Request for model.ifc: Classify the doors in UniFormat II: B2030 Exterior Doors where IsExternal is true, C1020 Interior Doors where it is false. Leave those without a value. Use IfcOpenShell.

First a look at what the model holds.

```python
import ifcopenshell
import ifcopenshell.util.element

model = ifcopenshell.open("model.ifc")
print(model.schema)
print("classifications:", [c.Name for c in model.by_type("IfcClassification")])
values = [ifcopenshell.util.element.get_pset(e, "Pset_DoorCommon", "IsExternal") for e in model.by_type("IfcDoor")]
for value in (True, False, None):
    print("IsExternal", value, values.count(value))
```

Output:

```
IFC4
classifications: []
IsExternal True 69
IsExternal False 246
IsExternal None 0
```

```python
import ifcopenshell
import ifcopenshell.api.classification
import ifcopenshell.util.element

model = ifcopenshell.open("model.ifc")

system = ifcopenshell.api.classification.add_classification(model, classification="UniFormat II")

doors = model.by_type("IfcDoor")
external = {e: ifcopenshell.util.element.get_pset(e, "Pset_DoorCommon", "IsExternal") for e in doors}
for flag, code, name in ((True, "B2030", "Exterior Doors"), (False, "C1020", "Interior Doors")):
    products = [e for e in doors if external[e] is flag]
    ifcopenshell.api.classification.add_reference(
        model, products=products, classification=system, identification=code, name=name
    )
    print(code, len(products))

model.write("model_updated.ifc")
```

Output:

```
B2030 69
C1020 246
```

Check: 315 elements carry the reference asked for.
